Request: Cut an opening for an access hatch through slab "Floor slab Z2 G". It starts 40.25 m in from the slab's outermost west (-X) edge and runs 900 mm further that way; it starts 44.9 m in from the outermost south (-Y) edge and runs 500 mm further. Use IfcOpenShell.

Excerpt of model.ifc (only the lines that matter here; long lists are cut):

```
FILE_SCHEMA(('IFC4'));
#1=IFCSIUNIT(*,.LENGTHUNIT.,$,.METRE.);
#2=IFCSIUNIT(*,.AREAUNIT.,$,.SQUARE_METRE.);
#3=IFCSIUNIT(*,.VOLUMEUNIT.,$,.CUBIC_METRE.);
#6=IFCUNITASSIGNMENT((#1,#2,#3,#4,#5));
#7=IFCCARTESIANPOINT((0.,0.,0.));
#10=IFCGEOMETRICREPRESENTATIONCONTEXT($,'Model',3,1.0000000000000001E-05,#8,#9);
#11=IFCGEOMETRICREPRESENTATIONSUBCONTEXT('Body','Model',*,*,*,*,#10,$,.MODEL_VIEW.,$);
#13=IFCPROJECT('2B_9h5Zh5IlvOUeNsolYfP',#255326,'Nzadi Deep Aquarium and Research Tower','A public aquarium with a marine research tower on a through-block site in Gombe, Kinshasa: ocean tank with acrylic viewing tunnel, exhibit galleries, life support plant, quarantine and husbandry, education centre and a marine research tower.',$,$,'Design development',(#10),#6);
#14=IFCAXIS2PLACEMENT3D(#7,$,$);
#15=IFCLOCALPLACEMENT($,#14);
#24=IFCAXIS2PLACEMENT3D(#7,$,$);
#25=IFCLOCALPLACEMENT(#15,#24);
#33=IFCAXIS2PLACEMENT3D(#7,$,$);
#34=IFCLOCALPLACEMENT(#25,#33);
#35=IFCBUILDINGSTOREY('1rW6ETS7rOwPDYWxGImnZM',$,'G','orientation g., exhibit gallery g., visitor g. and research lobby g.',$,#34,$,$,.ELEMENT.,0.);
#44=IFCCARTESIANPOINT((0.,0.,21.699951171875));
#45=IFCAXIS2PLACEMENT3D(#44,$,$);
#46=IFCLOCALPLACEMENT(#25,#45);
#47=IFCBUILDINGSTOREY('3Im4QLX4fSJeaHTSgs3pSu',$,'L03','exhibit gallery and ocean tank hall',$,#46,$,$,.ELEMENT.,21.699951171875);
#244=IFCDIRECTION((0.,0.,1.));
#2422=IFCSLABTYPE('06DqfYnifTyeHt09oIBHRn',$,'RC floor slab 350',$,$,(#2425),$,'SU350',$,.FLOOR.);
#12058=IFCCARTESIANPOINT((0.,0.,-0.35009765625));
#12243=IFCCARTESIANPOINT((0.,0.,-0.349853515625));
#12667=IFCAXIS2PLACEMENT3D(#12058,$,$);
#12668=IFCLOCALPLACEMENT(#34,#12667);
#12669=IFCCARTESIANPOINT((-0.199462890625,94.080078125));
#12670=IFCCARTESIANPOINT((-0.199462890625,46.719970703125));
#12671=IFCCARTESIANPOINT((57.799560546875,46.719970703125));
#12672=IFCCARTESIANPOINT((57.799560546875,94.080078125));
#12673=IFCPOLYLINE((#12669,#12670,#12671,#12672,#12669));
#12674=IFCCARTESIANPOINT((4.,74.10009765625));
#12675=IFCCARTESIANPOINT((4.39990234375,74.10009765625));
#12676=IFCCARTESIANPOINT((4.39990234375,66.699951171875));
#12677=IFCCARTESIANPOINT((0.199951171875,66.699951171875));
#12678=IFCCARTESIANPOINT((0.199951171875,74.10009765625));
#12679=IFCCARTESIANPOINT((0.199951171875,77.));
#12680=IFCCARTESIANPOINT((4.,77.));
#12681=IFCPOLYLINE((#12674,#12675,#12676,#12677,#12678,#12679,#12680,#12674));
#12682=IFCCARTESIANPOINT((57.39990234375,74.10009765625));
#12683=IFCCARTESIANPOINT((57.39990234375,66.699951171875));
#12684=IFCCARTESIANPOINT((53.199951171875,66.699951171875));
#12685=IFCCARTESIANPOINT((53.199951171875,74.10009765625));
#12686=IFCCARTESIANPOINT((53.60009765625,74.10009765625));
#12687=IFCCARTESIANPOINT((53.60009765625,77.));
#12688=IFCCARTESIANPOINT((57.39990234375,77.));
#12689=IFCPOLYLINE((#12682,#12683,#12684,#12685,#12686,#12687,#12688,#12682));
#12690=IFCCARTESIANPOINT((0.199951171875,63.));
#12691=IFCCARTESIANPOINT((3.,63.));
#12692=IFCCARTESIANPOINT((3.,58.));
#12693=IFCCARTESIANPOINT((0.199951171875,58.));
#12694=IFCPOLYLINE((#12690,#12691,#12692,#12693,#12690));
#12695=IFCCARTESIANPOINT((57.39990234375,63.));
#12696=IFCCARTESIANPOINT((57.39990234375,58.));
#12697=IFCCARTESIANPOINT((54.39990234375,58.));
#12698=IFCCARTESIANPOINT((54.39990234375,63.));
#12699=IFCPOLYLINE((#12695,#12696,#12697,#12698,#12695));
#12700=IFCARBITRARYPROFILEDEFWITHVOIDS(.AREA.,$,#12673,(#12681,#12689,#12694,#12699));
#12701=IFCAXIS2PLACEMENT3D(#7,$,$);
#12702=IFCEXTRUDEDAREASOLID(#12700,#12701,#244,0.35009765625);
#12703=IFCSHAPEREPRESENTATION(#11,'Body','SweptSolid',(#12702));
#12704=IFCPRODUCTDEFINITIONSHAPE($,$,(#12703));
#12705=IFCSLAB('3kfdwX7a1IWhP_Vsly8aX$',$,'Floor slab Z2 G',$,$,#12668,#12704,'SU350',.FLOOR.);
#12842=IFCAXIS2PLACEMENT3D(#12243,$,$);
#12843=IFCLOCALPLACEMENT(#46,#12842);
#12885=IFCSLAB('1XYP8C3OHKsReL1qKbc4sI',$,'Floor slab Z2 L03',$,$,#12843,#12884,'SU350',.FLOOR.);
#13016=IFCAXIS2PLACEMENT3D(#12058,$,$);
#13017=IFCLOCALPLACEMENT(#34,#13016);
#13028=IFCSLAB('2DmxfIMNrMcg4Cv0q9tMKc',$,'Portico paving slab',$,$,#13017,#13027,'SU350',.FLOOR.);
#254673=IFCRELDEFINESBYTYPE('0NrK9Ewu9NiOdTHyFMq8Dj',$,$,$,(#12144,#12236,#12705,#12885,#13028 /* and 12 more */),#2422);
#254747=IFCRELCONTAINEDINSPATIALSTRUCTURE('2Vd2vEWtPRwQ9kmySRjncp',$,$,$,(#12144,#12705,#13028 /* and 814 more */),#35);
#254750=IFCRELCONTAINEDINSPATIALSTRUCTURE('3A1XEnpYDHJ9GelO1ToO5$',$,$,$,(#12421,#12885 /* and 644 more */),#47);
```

```python
import numpy as np
import ifcopenshell
import ifcopenshell.api.feature
import ifcopenshell.api.geometry
import ifcopenshell.api.root
import ifcopenshell.geom
import ifcopenshell.util.placement
import ifcopenshell.util.representation
import ifcopenshell.util.shape
import ifcopenshell.util.unit

model = ifcopenshell.open("model.ifc")
unit_scale = ifcopenshell.util.unit.calculate_unit_scale(model)
settings = ifcopenshell.geom.settings()


def volume(element):
    """Net volume in cubic metres, openings subtracted."""
    shape = ifcopenshell.geom.create_shape(settings, element)
    return ifcopenshell.util.shape.get_volume(shape.geometry)


slab = model.by_id(12705)
before = volume(slab)

# Extent in the slab's own axes, in metres. The edges named are its -X and -Y sides.
slab_shape = ifcopenshell.geom.create_shape(settings, slab)
vertices = ifcopenshell.util.shape.get_vertices(slab_shape.geometry)
x_min, y_min, bottom = vertices.min(axis=0)
top = vertices[:, 2].max()

opening = ifcopenshell.api.root.create_entity(model, ifc_class="IfcOpeningElement", name="Access hatch opening", predefined_type="OPENING")
context = ifcopenshell.util.representation.get_context(model, "Model", "Body", "MODEL_VIEW")
width, depth = 0.9, 0.5
outline = [(0.0, 0.0), (width, 0.0), (width, depth), (0.0, depth), (0.0, 0.0)]
# Overshoot both faces by 50 mm so the cut is clean.
shape = ifcopenshell.api.geometry.add_slab_representation(
    model, context=context, depth=top - bottom + 0.1, polyline=outline
)
ifcopenshell.api.geometry.assign_representation(model, product=opening, representation=shape)

matrix = ifcopenshell.util.placement.get_local_placement(slab.ObjectPlacement)
matrix[:, 3] = matrix @ np.append(np.array([x_min + 40.25, y_min + 44.9, bottom - 0.05]) / unit_scale, 1.0)
ifcopenshell.api.geometry.edit_object_placement(model, product=opening, matrix=matrix, is_si=False)
ifcopenshell.api.feature.add_feature(model, feature=opening, element=slab)

after = volume(slab)

print(f"slab volume {before:.3f} -> {after:.3f} m3")

model.write("model_v2.ifc")
```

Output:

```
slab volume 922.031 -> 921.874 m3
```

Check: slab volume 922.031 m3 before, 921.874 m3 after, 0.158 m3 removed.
